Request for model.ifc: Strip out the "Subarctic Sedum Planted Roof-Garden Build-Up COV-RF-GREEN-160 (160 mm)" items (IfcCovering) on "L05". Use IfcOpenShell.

First a look at what the model holds.

```python
import ifcopenshell
import ifcopenshell.util.element

model = ifcopenshell.open("model.ifc")
print(model.schema)
storey = next(s for s in model.by_type("IfcBuildingStorey") if s.Name == "L05")
coverings = [e for e in ifcopenshell.util.element.get_decomposition(storey) if e.is_a("IfcCovering")]
seen = {}
for e in coverings:
    element_type = ifcopenshell.util.element.get_type(e)
    name = element_type.Name if element_type not in (None, e) else None
    seen[name] = seen.get(name, 0) + 1
for name, count in sorted(seen.items(), key=str):
    print(count, "x", name)
```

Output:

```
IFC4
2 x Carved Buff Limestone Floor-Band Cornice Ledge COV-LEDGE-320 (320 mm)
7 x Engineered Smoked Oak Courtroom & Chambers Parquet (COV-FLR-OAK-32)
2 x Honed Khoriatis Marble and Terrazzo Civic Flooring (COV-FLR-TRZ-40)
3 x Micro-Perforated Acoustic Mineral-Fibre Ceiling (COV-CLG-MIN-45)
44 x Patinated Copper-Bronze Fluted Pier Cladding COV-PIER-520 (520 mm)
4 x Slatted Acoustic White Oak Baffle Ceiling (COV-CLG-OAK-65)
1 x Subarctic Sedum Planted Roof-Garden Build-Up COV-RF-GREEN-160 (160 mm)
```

```python
import ifcopenshell
import ifcopenshell.api.root
import ifcopenshell.util.element

model = ifcopenshell.open("model.ifc")

storey = next(s for s in model.by_type("IfcBuildingStorey") if s.Name == "L05")
coverings = [e for e in ifcopenshell.util.element.get_decomposition(storey) if e.is_a("IfcCovering")]
targets = [e for e in coverings if (t := ifcopenshell.util.element.get_type(e)) not in (None, e) and t.Name == "Subarctic Sedum Planted Roof-Garden Build-Up COV-RF-GREEN-160 (160 mm)"]

for e in targets:
    ifcopenshell.api.root.remove_product(model, product=e)
print(len(targets), "removed")

model.write("model-out.ifc")
```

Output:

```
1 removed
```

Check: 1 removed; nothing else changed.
